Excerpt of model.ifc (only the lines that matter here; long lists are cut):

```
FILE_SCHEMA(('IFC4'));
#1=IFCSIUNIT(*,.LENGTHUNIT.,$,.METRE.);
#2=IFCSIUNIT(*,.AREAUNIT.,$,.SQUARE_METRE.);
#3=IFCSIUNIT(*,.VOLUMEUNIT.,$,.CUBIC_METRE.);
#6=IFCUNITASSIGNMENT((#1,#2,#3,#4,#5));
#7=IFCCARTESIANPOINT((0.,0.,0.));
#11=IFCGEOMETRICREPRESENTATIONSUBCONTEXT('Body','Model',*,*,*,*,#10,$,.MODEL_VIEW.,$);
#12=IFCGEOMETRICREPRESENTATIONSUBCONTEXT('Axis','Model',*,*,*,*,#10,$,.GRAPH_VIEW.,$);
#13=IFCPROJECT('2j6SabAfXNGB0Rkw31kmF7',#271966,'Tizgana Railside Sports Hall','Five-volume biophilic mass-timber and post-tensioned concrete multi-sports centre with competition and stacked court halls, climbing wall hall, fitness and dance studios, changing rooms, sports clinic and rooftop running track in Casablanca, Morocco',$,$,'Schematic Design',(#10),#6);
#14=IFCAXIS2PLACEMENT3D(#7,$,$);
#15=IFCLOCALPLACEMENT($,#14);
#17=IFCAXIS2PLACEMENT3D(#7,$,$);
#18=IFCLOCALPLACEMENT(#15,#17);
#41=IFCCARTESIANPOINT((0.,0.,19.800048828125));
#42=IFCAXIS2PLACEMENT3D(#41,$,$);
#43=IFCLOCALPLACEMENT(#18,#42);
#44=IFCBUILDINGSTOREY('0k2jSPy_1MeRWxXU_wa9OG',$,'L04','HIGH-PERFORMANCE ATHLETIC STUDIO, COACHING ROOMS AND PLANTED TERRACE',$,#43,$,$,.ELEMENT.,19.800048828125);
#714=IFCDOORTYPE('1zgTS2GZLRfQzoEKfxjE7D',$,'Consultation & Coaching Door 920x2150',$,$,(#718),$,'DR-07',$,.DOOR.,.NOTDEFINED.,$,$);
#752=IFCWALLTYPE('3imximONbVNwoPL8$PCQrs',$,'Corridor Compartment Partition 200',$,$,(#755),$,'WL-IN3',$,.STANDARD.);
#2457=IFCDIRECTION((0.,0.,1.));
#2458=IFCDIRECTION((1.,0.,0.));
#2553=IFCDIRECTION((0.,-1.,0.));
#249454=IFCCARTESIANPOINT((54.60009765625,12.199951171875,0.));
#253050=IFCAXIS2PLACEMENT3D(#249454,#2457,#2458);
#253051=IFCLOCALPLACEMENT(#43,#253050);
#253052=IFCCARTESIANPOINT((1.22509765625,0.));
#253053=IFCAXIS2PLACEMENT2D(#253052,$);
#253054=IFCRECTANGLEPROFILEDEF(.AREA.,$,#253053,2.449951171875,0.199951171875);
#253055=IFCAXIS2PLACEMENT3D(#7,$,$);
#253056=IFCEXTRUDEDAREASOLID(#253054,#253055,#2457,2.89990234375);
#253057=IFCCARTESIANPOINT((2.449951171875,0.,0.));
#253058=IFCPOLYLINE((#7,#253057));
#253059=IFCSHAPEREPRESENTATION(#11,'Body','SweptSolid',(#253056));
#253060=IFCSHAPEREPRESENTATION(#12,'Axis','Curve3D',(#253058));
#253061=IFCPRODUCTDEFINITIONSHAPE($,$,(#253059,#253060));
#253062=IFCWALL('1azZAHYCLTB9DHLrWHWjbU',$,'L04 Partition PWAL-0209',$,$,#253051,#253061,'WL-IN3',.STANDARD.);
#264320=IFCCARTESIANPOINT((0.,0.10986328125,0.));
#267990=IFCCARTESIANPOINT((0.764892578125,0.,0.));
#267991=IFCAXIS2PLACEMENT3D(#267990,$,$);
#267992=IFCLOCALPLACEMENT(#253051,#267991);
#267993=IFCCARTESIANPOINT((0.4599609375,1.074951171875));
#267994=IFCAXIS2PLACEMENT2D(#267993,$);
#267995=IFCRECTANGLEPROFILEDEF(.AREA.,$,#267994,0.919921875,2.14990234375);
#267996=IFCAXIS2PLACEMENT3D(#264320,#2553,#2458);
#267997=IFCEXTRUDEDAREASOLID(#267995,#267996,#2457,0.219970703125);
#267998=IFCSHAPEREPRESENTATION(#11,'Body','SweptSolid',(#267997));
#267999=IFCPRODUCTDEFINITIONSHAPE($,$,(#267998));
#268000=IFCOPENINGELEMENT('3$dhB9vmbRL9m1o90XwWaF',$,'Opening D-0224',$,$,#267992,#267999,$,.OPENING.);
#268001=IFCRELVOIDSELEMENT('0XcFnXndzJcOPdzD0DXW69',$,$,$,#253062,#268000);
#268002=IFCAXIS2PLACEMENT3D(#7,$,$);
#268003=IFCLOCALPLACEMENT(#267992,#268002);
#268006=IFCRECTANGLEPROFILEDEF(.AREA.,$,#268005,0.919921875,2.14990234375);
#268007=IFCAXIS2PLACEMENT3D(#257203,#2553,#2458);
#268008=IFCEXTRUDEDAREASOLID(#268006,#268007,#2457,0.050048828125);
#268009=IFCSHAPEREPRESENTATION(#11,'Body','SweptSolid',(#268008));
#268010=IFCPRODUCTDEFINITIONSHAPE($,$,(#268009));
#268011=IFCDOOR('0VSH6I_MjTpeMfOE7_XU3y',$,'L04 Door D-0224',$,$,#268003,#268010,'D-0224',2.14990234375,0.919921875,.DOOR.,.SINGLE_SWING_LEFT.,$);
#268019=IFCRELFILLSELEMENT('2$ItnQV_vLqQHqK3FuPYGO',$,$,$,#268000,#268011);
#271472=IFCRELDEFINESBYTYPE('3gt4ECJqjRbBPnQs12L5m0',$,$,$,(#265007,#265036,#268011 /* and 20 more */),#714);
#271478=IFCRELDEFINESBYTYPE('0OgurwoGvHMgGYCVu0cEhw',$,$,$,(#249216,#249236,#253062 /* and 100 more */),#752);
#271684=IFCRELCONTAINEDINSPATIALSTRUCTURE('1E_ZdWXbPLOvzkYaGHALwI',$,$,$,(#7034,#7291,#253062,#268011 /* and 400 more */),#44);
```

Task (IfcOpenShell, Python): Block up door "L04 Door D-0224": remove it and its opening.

```python
import ifcopenshell
import ifcopenshell.api.feature
import ifcopenshell.api.root
import ifcopenshell.geom
import ifcopenshell.util.shape

model = ifcopenshell.open("model.ifc")
settings = ifcopenshell.geom.settings()


def volume(element):
    """Net volume in cubic metres, openings subtracted."""
    shape = ifcopenshell.geom.create_shape(settings, element)
    return ifcopenshell.util.shape.get_volume(shape.geometry)


door = model.by_guid("0VSH6I_MjTpeMfOE7_XU3y")
opening = door.FillsVoids[0].RelatingOpeningElement
wall = opening.VoidsElements[0].RelatingBuildingElement
before = volume(wall)

ifcopenshell.api.root.remove_product(model, product=door)
ifcopenshell.api.feature.remove_feature(model, feature=opening)

after = volume(wall)

print(f"wall volume {before:.3f} -> {after:.3f} m3")

model.write("model-out.ifc")
```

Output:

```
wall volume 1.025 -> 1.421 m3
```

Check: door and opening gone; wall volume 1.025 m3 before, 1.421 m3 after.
